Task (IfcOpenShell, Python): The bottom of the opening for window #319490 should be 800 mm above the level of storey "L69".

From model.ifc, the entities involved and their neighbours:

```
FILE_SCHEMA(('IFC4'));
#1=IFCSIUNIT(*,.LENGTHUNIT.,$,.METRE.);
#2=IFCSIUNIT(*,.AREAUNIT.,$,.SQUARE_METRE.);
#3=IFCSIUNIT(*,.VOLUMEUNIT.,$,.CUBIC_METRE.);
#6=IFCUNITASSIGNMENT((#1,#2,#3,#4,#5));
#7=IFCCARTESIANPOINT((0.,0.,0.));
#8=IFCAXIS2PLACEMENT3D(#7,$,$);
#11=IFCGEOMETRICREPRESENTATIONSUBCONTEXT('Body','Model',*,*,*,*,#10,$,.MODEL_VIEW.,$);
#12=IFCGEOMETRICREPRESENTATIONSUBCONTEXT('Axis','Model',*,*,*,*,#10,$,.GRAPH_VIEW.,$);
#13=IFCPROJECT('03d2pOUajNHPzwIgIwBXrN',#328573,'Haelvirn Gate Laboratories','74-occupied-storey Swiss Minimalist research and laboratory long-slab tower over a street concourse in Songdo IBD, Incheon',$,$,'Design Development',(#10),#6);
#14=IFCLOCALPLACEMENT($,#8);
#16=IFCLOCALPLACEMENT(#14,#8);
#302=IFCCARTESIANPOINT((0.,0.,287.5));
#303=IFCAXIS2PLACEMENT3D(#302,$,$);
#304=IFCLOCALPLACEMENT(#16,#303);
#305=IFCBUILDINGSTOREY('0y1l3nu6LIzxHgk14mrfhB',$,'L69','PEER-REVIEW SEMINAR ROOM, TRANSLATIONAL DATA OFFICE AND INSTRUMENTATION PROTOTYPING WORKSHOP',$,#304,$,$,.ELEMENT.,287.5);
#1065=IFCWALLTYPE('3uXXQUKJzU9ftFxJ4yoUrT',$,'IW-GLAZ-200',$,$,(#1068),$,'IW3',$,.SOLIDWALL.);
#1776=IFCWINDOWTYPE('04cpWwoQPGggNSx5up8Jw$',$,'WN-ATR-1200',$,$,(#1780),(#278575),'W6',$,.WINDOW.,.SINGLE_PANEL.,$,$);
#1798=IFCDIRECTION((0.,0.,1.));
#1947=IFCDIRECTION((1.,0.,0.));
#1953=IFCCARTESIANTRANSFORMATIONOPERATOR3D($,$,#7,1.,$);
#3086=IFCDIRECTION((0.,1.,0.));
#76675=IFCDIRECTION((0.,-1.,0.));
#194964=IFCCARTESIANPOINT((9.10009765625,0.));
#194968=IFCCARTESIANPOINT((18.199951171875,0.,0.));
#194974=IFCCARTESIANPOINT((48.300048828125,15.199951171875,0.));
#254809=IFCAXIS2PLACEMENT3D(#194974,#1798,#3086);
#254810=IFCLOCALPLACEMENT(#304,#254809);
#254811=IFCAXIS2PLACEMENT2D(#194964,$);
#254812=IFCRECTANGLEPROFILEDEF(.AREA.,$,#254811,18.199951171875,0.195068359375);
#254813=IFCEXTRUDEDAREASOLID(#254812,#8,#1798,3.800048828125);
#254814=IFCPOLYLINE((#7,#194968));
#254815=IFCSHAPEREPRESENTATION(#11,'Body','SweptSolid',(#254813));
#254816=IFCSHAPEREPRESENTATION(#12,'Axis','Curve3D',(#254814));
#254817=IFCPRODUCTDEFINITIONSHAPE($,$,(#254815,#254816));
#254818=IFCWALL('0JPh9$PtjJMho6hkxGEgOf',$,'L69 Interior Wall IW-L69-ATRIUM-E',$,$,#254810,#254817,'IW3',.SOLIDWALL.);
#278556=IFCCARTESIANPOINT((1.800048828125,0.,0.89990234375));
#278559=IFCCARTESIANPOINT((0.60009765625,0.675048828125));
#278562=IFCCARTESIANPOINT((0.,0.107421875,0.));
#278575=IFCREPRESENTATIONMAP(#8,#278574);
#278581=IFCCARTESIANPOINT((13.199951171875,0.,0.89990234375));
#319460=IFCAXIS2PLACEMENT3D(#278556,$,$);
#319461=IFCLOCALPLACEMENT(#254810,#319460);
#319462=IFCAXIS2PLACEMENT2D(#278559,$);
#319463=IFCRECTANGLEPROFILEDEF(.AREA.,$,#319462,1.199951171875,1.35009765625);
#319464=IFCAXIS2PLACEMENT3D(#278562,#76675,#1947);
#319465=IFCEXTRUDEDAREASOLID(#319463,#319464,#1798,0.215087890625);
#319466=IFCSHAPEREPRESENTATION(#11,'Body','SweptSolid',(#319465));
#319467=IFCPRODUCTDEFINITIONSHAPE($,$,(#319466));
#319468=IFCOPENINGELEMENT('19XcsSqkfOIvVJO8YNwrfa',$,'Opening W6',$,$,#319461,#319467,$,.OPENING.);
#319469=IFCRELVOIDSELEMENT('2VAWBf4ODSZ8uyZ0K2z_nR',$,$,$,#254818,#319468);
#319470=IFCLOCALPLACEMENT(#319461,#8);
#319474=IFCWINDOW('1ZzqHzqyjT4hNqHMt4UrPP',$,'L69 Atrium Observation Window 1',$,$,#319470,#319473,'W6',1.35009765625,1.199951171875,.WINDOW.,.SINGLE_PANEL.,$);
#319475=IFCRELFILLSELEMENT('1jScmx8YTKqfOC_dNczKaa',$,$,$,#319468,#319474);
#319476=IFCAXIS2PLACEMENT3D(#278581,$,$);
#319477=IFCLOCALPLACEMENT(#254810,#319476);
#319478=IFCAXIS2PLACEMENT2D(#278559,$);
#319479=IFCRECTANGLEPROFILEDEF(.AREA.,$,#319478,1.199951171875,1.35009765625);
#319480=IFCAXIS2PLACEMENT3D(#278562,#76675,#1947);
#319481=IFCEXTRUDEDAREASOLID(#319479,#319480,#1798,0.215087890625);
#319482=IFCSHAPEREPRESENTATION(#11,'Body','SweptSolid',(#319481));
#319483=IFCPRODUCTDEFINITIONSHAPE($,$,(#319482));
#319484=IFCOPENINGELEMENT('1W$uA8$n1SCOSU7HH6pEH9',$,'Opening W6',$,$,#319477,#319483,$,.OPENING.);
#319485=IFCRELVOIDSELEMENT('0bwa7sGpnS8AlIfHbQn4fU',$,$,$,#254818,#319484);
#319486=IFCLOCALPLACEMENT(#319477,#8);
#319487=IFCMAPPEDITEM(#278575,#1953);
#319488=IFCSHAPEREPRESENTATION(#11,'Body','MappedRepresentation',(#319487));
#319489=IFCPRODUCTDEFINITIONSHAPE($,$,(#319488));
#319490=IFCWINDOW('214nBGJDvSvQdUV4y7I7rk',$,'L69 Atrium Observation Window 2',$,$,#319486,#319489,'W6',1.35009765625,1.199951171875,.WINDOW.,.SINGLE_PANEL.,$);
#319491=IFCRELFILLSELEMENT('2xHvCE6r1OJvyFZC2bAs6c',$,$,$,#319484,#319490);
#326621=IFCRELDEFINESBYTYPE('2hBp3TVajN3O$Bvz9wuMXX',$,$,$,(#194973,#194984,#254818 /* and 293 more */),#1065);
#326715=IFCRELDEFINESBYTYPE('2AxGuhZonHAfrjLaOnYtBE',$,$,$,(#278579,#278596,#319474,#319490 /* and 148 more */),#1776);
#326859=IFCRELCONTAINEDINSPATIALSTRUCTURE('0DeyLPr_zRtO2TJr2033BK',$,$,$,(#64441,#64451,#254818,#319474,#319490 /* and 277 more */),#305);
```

```python
import numpy as np
import ifcopenshell
import ifcopenshell.api.geometry
import ifcopenshell.geom
import ifcopenshell.util.element
import ifcopenshell.util.placement
import ifcopenshell.util.shape
import ifcopenshell.util.unit

model = ifcopenshell.open("model.ifc")
unit_scale = ifcopenshell.util.unit.calculate_unit_scale(model)

window = model.by_guid("214nBGJDvSvQdUV4y7I7rk")
opening = window.FillsVoids[0].RelatingOpeningElement
storey = ifcopenshell.util.element.get_container(window, ifc_class="IfcBuildingStorey")
level = ifcopenshell.util.placement.get_local_placement(storey.ObjectPlacement)[2, 3]

# The opening's origin need not be at the sill, so measure its lowest point.
shape = ifcopenshell.geom.create_shape(ifcopenshell.geom.settings(), opening)
bottom = ifcopenshell.util.shape.get_shape_bottom_elevation(shape, shape.geometry) / unit_scale
dz = level + 0.8 - bottom

shift = np.array([0.0, 0.0, dz])
# The window is placed relative to its opening, so it follows when the opening moves.
matrix = ifcopenshell.util.placement.get_local_placement(opening.ObjectPlacement)
matrix[:3, 3] += shift
ifcopenshell.api.geometry.edit_object_placement(
    model, product=opening, matrix=matrix, is_si=False, should_transform_children=True
)

print(f"moved by {dz * unit_scale:+.3f} m")

model.write("model-out.ifc")
```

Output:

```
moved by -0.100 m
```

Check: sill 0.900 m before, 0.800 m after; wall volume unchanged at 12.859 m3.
